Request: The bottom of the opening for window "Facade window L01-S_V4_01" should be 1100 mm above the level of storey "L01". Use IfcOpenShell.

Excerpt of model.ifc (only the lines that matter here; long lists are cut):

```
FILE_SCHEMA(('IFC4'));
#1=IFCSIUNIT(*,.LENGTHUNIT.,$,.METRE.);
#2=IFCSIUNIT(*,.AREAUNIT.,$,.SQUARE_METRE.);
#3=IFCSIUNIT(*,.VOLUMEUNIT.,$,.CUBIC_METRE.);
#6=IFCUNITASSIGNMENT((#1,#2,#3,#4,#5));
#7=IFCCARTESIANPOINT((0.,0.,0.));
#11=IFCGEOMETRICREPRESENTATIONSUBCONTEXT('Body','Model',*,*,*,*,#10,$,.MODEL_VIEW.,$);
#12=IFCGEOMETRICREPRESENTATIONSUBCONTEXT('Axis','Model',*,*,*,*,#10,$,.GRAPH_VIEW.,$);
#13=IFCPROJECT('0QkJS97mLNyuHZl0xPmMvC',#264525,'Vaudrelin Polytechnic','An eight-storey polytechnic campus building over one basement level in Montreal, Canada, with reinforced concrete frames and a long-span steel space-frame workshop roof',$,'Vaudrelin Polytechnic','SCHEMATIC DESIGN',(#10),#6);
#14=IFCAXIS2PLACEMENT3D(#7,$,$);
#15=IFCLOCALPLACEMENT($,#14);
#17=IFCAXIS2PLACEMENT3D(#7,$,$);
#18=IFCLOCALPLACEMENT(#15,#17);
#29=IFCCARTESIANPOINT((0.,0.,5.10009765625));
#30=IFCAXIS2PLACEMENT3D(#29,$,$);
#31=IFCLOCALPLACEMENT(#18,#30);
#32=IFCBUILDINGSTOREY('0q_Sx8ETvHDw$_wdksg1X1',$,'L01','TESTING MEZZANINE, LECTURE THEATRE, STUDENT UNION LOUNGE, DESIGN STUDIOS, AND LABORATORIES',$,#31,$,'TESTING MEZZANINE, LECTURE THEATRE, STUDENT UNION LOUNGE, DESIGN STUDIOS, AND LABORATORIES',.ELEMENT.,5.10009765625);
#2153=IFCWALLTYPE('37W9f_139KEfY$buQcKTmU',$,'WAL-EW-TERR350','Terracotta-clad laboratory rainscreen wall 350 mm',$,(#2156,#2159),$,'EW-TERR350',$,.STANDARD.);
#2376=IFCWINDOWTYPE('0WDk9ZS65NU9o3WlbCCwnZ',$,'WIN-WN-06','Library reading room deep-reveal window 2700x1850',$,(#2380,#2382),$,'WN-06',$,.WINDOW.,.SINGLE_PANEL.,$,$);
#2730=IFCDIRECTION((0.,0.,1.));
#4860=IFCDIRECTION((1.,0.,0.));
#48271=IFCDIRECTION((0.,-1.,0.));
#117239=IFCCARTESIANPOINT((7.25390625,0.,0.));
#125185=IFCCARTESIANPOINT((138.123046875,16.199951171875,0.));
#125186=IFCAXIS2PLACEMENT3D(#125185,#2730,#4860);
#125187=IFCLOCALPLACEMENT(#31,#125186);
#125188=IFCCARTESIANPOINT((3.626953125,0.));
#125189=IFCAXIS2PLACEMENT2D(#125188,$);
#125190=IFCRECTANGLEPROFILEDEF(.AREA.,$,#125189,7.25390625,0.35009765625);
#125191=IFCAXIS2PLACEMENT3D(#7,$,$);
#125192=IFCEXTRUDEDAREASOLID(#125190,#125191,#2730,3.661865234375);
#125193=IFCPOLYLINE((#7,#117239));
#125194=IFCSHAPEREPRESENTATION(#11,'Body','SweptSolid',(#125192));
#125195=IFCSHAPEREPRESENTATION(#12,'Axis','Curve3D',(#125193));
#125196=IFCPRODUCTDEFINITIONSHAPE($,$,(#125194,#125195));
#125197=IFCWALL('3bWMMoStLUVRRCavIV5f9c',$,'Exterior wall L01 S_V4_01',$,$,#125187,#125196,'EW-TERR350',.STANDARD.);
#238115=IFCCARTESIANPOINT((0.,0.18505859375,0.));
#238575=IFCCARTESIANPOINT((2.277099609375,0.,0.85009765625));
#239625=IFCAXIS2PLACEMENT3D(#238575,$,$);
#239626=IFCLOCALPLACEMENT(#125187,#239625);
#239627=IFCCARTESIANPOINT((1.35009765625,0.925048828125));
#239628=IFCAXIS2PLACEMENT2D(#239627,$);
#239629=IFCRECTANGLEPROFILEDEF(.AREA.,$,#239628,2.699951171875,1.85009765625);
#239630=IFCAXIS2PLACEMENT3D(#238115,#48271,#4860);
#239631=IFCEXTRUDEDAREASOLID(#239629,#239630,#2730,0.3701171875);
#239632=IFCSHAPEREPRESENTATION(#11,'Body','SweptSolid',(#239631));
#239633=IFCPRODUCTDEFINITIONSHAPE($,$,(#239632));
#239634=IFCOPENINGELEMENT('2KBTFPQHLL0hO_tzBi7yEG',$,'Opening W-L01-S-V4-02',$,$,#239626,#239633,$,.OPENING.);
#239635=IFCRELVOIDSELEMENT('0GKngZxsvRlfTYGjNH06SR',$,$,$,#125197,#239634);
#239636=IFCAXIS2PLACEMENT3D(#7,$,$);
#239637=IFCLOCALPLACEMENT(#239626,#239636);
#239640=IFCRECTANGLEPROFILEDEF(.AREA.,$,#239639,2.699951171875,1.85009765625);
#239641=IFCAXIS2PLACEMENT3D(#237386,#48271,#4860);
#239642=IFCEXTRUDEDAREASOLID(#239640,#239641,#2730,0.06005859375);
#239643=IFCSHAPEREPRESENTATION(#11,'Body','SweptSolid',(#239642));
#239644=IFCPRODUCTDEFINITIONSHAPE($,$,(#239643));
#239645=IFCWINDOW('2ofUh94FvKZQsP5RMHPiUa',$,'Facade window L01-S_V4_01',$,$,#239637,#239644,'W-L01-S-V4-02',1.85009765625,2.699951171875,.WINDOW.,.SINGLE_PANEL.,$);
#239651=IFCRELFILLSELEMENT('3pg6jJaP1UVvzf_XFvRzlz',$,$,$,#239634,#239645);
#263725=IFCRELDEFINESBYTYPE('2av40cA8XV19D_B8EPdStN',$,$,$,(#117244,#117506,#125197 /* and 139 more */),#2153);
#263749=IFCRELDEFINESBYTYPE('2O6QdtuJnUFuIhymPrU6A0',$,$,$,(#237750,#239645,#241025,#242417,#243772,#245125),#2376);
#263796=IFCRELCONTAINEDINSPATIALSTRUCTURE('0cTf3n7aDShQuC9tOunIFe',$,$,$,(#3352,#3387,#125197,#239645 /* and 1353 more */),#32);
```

```python
import numpy as np
import ifcopenshell
import ifcopenshell.api.geometry
import ifcopenshell.geom
import ifcopenshell.util.element
import ifcopenshell.util.placement
import ifcopenshell.util.shape
import ifcopenshell.util.unit

model = ifcopenshell.open("model.ifc")
unit_scale = ifcopenshell.util.unit.calculate_unit_scale(model)

window = model.by_guid("2ofUh94FvKZQsP5RMHPiUa")
opening = window.FillsVoids[0].RelatingOpeningElement
storey = ifcopenshell.util.element.get_container(window, ifc_class="IfcBuildingStorey")
level = ifcopenshell.util.placement.get_local_placement(storey.ObjectPlacement)[2, 3]

# The opening's origin need not be at the sill, so measure its lowest point.
shape = ifcopenshell.geom.create_shape(ifcopenshell.geom.settings(), opening)
bottom = ifcopenshell.util.shape.get_shape_bottom_elevation(shape, shape.geometry) / unit_scale
dz = level + 1.1 / unit_scale - bottom

shift = np.array([0.0, 0.0, dz])
# The window is placed relative to its opening, so it follows when the opening moves.
matrix = ifcopenshell.util.placement.get_local_placement(opening.ObjectPlacement)
matrix[:3, 3] += shift
ifcopenshell.api.geometry.edit_object_placement(
    model, product=opening, matrix=matrix, is_si=False, should_transform_children=True
)

print(f"moved by {dz * unit_scale:+.3f} m")

model.write("model_edited.ifc")
```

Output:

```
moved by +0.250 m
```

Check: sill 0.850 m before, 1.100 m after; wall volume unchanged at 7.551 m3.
